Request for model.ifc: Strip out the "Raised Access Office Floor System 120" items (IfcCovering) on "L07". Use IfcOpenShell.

First a look at what the model holds.

```python
import ifcopenshell
import ifcopenshell.util.element

model = ifcopenshell.open("model.ifc")
print(model.schema)
storey = next(s for s in model.by_type("IfcBuildingStorey") if s.Name == "L07")
coverings = [e for e in ifcopenshell.util.element.get_decomposition(storey) if e.is_a("IfcCovering")]
seen = {}
for e in coverings:
    element_type = ifcopenshell.util.element.get_type(e)
    name = element_type.Name if element_type not in (None, e) else None
    seen[name] = seen.get(name, 0) + 1
for name, count in sorted(seen.items(), key=str):
    print(count, "x", name)
```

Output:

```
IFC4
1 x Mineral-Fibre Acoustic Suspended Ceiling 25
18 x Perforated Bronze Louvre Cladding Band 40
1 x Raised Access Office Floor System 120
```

```python
import ifcopenshell
import ifcopenshell.api.root
import ifcopenshell.util.element

model = ifcopenshell.open("model.ifc")

storey = next(s for s in model.by_type("IfcBuildingStorey") if s.Name == "L07")
coverings = [e for e in ifcopenshell.util.element.get_decomposition(storey) if e.is_a("IfcCovering")]
targets = [e for e in coverings if (t := ifcopenshell.util.element.get_type(e)) not in (None, e) and t.Name == "Raised Access Office Floor System 120"]

for e in targets:
    ifcopenshell.api.root.remove_product(model, product=e)
print(len(targets), "removed")

model.write("model-out.ifc")
```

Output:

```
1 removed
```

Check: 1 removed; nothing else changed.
